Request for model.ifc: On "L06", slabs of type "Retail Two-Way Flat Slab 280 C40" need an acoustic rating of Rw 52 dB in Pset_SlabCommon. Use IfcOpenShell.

First a look at what the model holds.

```python
import ifcopenshell
import ifcopenshell.util.element

model = ifcopenshell.open("model.ifc")
print(model.schema)
storey = next(s for s in model.by_type("IfcBuildingStorey") if s.Name == "L06")
slabs = [e for e in ifcopenshell.util.element.get_decomposition(storey) if e.is_a("IfcSlab")]
seen = {}
for e in slabs:
    element_type = ifcopenshell.util.element.get_type(e)
    key = (element_type.Name if element_type != e and element_type else None, ifcopenshell.util.element.get_pset(e, "Pset_SlabCommon", "AcousticRating"))
    seen[key] = seen.get(key, 0) + 1
for (name, value), count in sorted(seen.items(), key=str):
    print(count, "x", name, "|", value)
```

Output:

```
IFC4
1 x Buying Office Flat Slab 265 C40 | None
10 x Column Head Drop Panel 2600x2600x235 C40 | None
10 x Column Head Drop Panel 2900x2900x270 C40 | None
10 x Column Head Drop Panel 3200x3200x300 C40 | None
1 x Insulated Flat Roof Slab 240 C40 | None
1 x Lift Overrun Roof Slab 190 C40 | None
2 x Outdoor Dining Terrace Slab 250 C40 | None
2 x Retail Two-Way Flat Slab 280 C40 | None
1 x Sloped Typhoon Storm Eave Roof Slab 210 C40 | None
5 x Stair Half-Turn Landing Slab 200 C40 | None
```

```python
import ifcopenshell
import ifcopenshell.api.pset
import ifcopenshell.util.element

model = ifcopenshell.open("model.ifc")

storey = next(s for s in model.by_type("IfcBuildingStorey") if s.Name == "L06")
slabs = [e for e in ifcopenshell.util.element.get_decomposition(storey) if e.is_a("IfcSlab")]

count = 0
for e in slabs:
    element_type = ifcopenshell.util.element.get_type(e)
    if element_type in (None, e) or element_type.Name != "Retail Two-Way Flat Slab 280 C40":
        continue
    # add_pset returns the element's existing set when there is one.
    pset = ifcopenshell.api.pset.add_pset(model, product=e, name="Pset_SlabCommon")
    ifcopenshell.api.pset.edit_pset(model, pset=pset, properties={"AcousticRating": "Rw 52 dB"})
    count += 1

print(count, "slabs updated")

model.write("model_edited.ifc")
```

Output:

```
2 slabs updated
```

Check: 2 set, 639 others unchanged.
